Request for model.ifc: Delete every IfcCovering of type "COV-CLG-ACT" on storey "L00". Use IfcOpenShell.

First a look at what the model holds.

```python
import ifcopenshell
import ifcopenshell.util.element

model = ifcopenshell.open("model.ifc")
print(model.schema)
storey = next(s for s in model.by_type("IfcBuildingStorey") if s.Name == "L00")
coverings = [e for e in ifcopenshell.util.element.get_decomposition(storey) if e.is_a("IfcCovering")]
seen = {}
for e in coverings:
    element_type = ifcopenshell.util.element.get_type(e)
    name = element_type.Name if element_type not in (None, e) else None
    seen[name] = seen.get(name, 0) + 1
for name, count in sorted(seen.items(), key=str):
    print(count, "x", name)
```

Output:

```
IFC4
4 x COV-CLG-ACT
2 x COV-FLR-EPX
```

```python
import ifcopenshell
import ifcopenshell.api.root
import ifcopenshell.util.element

model = ifcopenshell.open("model.ifc")

storey = next(s for s in model.by_type("IfcBuildingStorey") if s.Name == "L00")
coverings = [e for e in ifcopenshell.util.element.get_decomposition(storey) if e.is_a("IfcCovering")]
targets = [e for e in coverings if (t := ifcopenshell.util.element.get_type(e)) not in (None, e) and t.Name == "COV-CLG-ACT"]

for e in targets:
    ifcopenshell.api.root.remove_product(model, product=e)
print(len(targets), "removed")

model.write("model_updated.ifc")
```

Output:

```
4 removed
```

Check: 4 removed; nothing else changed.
